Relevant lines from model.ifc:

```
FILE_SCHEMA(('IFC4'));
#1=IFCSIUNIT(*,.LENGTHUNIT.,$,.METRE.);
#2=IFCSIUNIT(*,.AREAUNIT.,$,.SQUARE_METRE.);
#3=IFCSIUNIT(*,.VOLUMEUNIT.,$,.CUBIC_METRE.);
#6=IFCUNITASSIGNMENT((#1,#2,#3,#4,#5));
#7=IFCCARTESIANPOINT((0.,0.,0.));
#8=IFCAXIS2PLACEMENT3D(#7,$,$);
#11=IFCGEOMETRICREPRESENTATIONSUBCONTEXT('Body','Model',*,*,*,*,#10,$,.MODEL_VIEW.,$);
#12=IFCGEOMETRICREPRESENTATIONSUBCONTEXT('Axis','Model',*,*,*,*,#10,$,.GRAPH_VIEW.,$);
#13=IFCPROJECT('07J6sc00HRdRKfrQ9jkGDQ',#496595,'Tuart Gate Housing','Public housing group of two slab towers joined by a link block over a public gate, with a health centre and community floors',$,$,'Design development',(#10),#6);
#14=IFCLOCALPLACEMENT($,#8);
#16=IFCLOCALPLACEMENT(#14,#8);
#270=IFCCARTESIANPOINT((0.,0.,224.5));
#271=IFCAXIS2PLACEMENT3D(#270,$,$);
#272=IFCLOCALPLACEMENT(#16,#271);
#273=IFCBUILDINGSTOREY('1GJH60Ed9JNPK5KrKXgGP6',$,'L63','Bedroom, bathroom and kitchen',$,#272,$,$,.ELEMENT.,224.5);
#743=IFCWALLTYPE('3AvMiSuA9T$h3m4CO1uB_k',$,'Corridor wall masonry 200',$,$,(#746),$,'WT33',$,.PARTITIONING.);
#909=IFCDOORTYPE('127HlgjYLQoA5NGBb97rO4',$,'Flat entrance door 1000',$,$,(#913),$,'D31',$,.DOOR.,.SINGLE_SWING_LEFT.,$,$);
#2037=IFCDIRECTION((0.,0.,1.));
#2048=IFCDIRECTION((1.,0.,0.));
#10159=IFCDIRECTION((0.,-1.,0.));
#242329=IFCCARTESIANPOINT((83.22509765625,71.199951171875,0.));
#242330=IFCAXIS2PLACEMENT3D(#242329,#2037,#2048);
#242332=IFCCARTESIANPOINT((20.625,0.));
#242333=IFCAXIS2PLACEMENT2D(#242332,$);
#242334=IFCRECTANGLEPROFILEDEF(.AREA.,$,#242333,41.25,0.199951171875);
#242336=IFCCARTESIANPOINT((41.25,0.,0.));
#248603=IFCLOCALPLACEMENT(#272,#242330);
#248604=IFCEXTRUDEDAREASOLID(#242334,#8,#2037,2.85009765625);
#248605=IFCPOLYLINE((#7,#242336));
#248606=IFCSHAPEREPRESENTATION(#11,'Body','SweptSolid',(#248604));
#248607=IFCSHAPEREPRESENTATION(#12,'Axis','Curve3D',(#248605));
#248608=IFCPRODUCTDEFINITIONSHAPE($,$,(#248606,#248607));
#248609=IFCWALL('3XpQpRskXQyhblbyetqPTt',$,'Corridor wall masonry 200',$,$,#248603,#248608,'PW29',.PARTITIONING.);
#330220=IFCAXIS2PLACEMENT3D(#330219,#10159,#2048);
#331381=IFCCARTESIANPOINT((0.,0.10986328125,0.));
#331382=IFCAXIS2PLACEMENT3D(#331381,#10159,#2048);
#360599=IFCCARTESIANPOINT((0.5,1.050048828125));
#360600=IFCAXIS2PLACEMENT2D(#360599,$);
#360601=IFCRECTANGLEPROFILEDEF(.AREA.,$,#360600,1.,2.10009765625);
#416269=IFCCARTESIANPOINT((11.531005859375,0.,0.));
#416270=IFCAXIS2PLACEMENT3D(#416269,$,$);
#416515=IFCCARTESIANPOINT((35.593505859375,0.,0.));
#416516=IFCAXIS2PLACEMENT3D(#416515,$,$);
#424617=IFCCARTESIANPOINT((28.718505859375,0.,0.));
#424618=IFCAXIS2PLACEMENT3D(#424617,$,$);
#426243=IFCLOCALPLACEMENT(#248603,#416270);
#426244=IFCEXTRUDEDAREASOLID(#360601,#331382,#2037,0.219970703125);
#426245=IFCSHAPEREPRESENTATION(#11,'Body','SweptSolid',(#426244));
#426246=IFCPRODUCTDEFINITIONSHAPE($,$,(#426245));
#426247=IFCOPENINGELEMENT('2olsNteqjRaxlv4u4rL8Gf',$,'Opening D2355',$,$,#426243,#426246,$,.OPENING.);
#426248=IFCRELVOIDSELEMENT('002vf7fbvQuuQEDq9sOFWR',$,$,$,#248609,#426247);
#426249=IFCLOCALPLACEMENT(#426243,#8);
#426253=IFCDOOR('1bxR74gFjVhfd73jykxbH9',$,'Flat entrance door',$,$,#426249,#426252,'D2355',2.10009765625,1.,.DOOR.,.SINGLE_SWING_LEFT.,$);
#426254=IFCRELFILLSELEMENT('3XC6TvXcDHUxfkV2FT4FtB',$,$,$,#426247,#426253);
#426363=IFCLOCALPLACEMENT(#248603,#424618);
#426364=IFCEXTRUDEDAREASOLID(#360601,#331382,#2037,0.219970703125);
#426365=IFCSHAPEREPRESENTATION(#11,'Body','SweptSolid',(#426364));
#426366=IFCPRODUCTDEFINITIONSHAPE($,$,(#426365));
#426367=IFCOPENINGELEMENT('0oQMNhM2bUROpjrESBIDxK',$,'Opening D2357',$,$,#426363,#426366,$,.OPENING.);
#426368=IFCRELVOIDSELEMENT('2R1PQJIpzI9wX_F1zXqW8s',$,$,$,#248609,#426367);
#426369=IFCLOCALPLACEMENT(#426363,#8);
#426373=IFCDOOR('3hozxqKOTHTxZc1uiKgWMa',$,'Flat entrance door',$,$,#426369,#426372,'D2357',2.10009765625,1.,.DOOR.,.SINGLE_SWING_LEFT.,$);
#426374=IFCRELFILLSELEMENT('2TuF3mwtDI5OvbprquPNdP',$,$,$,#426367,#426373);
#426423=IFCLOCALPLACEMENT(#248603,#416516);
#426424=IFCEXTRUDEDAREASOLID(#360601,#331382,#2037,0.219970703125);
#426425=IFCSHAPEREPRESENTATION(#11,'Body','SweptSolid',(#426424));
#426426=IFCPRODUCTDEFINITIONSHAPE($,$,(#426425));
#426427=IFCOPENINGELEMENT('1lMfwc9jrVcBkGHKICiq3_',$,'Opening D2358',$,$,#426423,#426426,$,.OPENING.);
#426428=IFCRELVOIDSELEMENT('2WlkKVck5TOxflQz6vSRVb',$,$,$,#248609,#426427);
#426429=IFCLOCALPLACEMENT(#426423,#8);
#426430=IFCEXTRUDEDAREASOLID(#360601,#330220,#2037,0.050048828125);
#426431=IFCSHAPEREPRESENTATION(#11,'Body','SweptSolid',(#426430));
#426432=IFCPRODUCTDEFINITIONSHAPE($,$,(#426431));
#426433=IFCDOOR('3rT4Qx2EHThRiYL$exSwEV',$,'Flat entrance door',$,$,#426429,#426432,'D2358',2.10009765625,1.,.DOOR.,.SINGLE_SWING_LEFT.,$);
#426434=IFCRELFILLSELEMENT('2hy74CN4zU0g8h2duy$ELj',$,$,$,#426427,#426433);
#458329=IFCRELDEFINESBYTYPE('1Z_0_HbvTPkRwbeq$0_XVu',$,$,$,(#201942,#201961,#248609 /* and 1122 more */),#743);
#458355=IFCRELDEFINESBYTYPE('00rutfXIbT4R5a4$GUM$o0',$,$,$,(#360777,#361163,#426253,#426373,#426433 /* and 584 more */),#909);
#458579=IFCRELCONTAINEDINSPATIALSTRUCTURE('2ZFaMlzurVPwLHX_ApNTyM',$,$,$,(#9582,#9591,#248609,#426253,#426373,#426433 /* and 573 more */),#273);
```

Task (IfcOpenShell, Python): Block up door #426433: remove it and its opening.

```python
import ifcopenshell
import ifcopenshell.api.feature
import ifcopenshell.api.root
import ifcopenshell.geom
import ifcopenshell.util.shape

model = ifcopenshell.open("model.ifc")
settings = ifcopenshell.geom.settings()


def volume(element):
    """Net volume in cubic metres, openings subtracted."""
    shape = ifcopenshell.geom.create_shape(settings, element)
    return ifcopenshell.util.shape.get_volume(shape.geometry)


door = model.by_guid("3rT4Qx2EHThRiYL$exSwEV")
opening = door.FillsVoids[0].RelatingOpeningElement
wall = opening.VoidsElements[0].RelatingBuildingElement
before = volume(wall)

ifcopenshell.api.root.remove_product(model, product=door)
ifcopenshell.api.feature.remove_feature(model, feature=opening)

after = volume(wall)

print(f"wall volume {before:.3f} -> {after:.3f} m3")

model.write("model-out.ifc")
```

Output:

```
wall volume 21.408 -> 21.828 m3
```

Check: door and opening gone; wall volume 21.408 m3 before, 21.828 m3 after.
